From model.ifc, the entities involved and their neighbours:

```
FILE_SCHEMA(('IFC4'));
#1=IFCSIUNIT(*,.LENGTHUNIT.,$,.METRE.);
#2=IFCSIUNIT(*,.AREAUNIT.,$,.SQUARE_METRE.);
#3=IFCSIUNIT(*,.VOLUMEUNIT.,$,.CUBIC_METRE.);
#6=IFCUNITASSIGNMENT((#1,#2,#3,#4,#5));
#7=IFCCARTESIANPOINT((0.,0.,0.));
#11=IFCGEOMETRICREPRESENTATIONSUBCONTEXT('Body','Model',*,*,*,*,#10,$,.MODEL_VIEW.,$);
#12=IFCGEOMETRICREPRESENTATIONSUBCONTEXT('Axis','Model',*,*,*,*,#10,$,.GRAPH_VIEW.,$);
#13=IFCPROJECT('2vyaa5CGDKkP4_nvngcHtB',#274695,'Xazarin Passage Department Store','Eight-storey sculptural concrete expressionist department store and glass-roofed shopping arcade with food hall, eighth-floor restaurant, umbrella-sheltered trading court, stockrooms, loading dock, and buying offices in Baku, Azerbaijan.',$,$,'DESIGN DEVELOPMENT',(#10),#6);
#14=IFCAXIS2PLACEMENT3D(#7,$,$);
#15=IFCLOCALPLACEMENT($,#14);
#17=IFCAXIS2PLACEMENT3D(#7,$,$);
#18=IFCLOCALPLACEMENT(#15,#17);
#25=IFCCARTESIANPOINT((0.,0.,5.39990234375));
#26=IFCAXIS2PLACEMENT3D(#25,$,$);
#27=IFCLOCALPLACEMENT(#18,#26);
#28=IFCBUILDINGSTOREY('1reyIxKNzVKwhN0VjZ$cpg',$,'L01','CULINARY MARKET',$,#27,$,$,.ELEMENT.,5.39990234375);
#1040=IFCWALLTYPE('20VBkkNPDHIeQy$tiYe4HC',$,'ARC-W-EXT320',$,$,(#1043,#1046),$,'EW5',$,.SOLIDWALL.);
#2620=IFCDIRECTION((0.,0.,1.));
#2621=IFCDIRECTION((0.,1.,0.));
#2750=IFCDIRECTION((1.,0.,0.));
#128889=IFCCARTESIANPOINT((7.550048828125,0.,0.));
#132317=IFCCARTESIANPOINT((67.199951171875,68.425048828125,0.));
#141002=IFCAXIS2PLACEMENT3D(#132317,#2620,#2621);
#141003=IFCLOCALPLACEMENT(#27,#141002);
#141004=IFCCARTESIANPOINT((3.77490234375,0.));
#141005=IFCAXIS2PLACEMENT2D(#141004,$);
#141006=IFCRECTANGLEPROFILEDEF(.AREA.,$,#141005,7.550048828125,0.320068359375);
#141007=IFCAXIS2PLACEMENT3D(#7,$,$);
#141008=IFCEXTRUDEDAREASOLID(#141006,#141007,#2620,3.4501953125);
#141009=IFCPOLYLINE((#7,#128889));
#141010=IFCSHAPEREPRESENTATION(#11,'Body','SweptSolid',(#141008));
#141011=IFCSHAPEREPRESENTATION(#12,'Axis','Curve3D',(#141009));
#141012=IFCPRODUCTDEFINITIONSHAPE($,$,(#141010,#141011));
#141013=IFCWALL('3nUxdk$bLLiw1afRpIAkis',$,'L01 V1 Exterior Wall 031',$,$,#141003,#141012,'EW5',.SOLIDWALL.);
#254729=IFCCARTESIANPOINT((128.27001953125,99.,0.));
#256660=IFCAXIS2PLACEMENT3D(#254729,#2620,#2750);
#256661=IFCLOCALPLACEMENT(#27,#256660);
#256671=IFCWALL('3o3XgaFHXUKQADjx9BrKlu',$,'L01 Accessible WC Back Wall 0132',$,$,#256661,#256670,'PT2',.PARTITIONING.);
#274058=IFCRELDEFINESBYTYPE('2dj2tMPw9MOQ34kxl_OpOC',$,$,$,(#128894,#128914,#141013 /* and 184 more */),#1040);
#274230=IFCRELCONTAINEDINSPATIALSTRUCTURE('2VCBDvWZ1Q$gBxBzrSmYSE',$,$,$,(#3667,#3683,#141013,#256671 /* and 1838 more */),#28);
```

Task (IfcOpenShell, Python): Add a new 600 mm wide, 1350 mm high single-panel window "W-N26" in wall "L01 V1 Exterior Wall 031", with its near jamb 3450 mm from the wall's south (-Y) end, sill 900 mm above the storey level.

```python
import numpy as np
import ifcopenshell
import ifcopenshell.api.feature
import ifcopenshell.api.geometry
import ifcopenshell.api.root
import ifcopenshell.api.spatial
import ifcopenshell.geom
import ifcopenshell.util.element
import ifcopenshell.util.placement
import ifcopenshell.util.representation
import ifcopenshell.util.shape
import ifcopenshell.util.unit

model = ifcopenshell.open("model.ifc")
unit_scale = ifcopenshell.util.unit.calculate_unit_scale(model)
settings = ifcopenshell.geom.settings()


def volume(element):
    """Net volume in cubic metres, openings subtracted."""
    shape = ifcopenshell.geom.create_shape(settings, element)
    return ifcopenshell.util.shape.get_volume(shape.geometry)


wall = model.by_id(141013)
storey = ifcopenshell.util.element.get_container(wall, ifc_class="IfcBuildingStorey")
context = ifcopenshell.util.representation.get_context(model, "Model", "Body", "MODEL_VIEW")
before = volume(wall)

width, height, from_end, sill = 0.6, 1.35, 3.45, 0.9  # metres

# The wall runs along its own X axis, and the end named is its -X end.
wall_shape = ifcopenshell.geom.create_shape(settings, wall)
x, y, z = ifcopenshell.util.shape.get_vertices(wall_shape.geometry).T
start = x.min() + from_end
face, thickness = float(y.min()), float(y.max() - y.min())
wall_matrix = ifcopenshell.util.placement.get_local_placement(wall.ObjectPlacement)
level = ifcopenshell.util.placement.get_local_placement(storey.ObjectPlacement)[2, 3]


def in_wall(x, y):
    """Placement at x, y metres in the wall's axes, at sill height."""
    matrix = wall_matrix.copy()
    matrix[:, 3] = wall_matrix @ np.array([x / unit_scale, y / unit_scale, 0.0, 1.0])
    matrix[2, 3] = level + sill / unit_scale
    return matrix


# Opening: a box that overshoots both wall faces by 50 mm.
opening = ifcopenshell.api.root.create_entity(model, ifc_class="IfcOpeningElement", predefined_type="OPENING")
box = ifcopenshell.api.geometry.add_wall_representation(
    model, context=context, length=width, height=height, thickness=thickness + 0.1
)
ifcopenshell.api.geometry.assign_representation(model, product=opening, representation=box)
ifcopenshell.api.geometry.edit_object_placement(model, product=opening, matrix=in_wall(start, face - 0.05), is_si=False)
ifcopenshell.api.feature.add_feature(model, feature=opening, element=wall)

window = ifcopenshell.api.root.create_entity(model, ifc_class="IfcWindow", name="W-N26", predefined_type="WINDOW")
window.OverallWidth, window.OverallHeight = width / unit_scale, height / unit_scale
window.PartitioningType = "SINGLE_PANEL"
body = ifcopenshell.api.geometry.add_window_representation(
    model,
    context=context,
    overall_width=window.OverallWidth,
    overall_height=window.OverallHeight,
    partition_type="SINGLE_PANEL",
)
ifcopenshell.api.geometry.assign_representation(model, product=window, representation=body)
ifcopenshell.api.spatial.assign_container(model, products=[window], relating_structure=storey)
ifcopenshell.api.feature.add_filling(model, opening=opening, element=window)

# Centre the window in the wall's thickness.
ifcopenshell.api.geometry.edit_object_placement(model, product=window, matrix=in_wall(start, face), is_si=False)
window_shape = ifcopenshell.geom.create_shape(settings, window)
depth = ifcopenshell.util.shape.get_vertices(window_shape.geometry)[:, 1]
offset = face + thickness / 2 - (depth.min() + depth.max()) / 2
ifcopenshell.api.geometry.edit_object_placement(model, product=window, matrix=in_wall(start, offset), is_si=False)

after = volume(wall)

print(f"wall volume {before:.3f} -> {after:.3f} m3")

model.write("model_rev.ifc")
```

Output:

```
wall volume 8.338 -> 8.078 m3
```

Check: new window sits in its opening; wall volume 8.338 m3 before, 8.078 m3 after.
